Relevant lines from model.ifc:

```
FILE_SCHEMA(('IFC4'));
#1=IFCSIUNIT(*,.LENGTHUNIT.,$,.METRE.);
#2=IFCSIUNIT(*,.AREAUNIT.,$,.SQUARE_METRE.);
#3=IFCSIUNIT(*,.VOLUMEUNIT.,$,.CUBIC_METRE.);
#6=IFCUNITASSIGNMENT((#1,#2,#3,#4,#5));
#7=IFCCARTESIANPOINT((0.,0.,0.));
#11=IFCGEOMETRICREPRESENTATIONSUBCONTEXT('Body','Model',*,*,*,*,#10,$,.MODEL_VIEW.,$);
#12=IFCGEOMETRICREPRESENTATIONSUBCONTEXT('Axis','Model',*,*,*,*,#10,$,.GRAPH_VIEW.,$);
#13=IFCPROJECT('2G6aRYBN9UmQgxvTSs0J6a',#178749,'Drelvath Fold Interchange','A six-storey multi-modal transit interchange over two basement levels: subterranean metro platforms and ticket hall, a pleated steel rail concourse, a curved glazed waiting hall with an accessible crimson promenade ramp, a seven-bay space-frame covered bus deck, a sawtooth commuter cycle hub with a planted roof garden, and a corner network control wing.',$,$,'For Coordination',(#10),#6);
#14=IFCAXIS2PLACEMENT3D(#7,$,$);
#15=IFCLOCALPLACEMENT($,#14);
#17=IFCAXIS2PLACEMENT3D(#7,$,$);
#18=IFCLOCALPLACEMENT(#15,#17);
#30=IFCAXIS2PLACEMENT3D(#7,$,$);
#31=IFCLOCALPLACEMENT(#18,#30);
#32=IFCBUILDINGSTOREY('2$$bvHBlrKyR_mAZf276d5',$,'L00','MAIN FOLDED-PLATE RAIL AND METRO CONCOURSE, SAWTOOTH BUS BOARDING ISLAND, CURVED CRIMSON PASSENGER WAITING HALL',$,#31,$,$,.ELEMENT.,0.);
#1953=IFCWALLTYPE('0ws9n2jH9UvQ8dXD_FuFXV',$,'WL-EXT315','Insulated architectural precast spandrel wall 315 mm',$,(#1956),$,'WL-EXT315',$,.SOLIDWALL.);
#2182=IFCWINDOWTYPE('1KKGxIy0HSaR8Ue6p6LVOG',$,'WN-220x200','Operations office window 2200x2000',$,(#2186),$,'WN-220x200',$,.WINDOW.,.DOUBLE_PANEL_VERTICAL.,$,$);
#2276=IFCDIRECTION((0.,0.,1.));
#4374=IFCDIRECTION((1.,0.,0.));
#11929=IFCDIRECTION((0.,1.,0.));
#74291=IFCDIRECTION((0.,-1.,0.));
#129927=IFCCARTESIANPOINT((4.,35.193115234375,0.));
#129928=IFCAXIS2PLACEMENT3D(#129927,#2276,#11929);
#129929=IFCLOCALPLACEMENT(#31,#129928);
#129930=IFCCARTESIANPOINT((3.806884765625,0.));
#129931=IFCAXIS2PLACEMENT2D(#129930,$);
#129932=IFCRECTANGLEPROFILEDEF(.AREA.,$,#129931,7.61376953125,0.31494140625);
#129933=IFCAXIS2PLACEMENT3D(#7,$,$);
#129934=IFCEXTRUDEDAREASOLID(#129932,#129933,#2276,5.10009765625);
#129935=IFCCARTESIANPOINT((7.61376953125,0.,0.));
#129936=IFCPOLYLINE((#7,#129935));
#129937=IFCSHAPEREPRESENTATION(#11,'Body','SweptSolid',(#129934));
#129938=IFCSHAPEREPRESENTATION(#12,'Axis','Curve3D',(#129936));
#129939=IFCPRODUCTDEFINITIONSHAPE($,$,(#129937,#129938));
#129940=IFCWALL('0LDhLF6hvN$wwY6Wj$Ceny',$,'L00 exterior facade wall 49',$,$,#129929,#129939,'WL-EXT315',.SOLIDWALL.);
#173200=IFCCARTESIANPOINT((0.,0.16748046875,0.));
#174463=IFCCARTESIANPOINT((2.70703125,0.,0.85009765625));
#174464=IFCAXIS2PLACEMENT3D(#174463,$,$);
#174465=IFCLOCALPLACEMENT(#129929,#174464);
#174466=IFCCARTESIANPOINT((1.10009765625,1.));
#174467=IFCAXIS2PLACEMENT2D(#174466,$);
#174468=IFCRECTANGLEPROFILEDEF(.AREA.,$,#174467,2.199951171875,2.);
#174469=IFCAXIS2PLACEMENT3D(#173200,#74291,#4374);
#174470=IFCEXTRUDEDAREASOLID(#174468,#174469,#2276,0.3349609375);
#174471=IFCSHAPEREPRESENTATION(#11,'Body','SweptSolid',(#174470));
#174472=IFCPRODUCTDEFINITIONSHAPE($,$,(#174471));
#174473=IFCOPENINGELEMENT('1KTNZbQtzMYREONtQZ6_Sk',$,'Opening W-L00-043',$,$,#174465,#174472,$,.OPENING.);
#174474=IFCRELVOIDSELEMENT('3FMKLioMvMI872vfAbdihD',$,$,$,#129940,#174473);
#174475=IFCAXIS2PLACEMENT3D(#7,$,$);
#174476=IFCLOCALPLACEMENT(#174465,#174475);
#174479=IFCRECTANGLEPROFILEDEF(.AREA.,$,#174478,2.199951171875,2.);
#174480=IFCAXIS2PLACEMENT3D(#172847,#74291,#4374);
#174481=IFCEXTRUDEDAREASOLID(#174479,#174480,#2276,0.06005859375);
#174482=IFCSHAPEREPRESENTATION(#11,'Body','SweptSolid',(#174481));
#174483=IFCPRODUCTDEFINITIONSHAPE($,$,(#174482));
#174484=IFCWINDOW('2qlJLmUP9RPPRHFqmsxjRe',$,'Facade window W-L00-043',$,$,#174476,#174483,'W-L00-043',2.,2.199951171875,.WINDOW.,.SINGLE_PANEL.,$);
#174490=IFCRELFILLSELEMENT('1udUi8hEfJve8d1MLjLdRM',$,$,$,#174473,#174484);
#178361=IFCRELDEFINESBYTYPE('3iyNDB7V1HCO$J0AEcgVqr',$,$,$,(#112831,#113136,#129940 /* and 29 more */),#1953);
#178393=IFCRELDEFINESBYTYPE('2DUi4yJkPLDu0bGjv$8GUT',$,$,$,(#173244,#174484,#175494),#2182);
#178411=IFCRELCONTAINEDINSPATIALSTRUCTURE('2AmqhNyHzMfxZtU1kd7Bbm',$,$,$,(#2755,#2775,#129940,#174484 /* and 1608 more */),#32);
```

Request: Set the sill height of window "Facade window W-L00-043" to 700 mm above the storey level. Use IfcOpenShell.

```python
import numpy as np
import ifcopenshell
import ifcopenshell.api.geometry
import ifcopenshell.geom
import ifcopenshell.util.element
import ifcopenshell.util.placement
import ifcopenshell.util.shape
import ifcopenshell.util.unit

model = ifcopenshell.open("model.ifc")
unit_scale = ifcopenshell.util.unit.calculate_unit_scale(model)

window = model.by_id(174484)
opening = window.FillsVoids[0].RelatingOpeningElement
storey = ifcopenshell.util.element.get_container(window, ifc_class="IfcBuildingStorey")
level = ifcopenshell.util.placement.get_local_placement(storey.ObjectPlacement)[2, 3]

# The opening's origin need not be at the sill, so measure its lowest point.
shape = ifcopenshell.geom.create_shape(ifcopenshell.geom.settings(), opening)
bottom = ifcopenshell.util.shape.get_shape_bottom_elevation(shape, shape.geometry) / unit_scale
dz = level + 0.7 - bottom

shift = np.array([0.0, 0.0, dz])
# The window is placed relative to its opening, so it follows when the opening moves.
matrix = ifcopenshell.util.placement.get_local_placement(opening.ObjectPlacement)
matrix[:3, 3] += shift
ifcopenshell.api.geometry.edit_object_placement(
    model, product=opening, matrix=matrix, is_si=False, should_transform_children=True
)

print(f"moved by {dz * unit_scale:+.3f} m")

model.write("model_edited.ifc")
```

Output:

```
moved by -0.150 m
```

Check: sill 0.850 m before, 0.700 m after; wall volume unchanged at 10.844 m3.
